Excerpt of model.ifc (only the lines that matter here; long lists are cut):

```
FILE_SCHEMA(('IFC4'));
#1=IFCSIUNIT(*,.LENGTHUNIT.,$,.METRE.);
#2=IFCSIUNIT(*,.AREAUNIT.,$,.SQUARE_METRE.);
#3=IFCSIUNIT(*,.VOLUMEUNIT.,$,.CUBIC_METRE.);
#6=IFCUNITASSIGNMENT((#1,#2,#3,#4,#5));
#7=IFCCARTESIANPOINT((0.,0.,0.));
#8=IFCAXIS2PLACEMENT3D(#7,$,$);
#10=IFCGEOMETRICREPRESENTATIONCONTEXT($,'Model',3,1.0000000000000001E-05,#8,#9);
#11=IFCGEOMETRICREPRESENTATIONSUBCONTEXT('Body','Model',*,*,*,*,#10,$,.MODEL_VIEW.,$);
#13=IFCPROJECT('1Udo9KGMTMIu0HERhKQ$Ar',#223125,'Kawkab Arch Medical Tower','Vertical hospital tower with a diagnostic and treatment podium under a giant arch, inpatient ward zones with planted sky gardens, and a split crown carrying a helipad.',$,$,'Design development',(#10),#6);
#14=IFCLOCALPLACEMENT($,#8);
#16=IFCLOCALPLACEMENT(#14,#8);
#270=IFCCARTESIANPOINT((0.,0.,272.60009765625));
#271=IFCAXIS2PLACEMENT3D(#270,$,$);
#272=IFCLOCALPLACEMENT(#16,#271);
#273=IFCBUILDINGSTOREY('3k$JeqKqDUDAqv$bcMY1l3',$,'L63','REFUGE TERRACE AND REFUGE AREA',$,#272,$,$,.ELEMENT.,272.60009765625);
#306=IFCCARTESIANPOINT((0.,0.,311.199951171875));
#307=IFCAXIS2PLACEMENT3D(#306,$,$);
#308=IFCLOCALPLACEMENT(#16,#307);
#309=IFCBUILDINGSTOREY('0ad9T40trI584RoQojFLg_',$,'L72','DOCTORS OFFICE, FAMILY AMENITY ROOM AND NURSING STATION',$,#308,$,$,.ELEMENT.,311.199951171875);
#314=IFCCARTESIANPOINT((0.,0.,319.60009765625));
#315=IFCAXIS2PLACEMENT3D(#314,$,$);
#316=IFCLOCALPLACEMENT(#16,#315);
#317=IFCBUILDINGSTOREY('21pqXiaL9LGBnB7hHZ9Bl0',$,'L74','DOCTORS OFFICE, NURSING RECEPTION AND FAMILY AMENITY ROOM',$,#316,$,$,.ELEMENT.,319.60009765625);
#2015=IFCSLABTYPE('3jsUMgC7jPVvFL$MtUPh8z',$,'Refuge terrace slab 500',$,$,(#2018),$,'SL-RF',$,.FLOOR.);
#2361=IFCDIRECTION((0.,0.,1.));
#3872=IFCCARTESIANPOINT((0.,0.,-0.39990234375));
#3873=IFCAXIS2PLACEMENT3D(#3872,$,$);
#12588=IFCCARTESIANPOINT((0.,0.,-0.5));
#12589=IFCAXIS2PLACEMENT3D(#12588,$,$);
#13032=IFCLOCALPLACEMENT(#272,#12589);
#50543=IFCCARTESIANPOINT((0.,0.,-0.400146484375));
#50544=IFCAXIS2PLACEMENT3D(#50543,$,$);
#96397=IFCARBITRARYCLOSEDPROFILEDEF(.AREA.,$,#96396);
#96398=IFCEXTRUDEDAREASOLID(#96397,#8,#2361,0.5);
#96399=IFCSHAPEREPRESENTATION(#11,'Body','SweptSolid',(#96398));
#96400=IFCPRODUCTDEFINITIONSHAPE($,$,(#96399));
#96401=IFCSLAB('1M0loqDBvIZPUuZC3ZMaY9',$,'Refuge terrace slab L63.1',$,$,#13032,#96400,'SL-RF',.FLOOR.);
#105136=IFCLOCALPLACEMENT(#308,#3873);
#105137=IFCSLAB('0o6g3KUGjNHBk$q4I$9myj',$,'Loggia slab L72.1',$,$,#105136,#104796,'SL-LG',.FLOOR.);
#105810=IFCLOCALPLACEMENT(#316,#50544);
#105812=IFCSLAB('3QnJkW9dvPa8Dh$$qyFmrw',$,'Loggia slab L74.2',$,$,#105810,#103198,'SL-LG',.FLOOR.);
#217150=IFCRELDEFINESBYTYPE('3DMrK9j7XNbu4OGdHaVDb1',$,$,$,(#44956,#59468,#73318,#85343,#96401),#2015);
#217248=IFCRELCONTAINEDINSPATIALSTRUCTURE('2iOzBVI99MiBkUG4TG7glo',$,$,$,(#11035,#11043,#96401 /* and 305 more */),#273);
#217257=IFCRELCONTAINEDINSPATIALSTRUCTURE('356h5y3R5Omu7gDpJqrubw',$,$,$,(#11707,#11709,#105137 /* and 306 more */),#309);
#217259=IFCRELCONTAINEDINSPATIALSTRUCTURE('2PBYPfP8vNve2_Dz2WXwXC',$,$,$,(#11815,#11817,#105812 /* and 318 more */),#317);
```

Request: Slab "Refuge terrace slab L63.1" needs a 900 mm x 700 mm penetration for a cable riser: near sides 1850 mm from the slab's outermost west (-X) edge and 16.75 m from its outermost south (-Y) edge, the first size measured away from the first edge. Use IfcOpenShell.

```python
import numpy as np
import ifcopenshell
import ifcopenshell.api.feature
import ifcopenshell.api.geometry
import ifcopenshell.api.root
import ifcopenshell.geom
import ifcopenshell.util.placement
import ifcopenshell.util.representation
import ifcopenshell.util.shape
import ifcopenshell.util.unit

model = ifcopenshell.open("model.ifc")
unit_scale = ifcopenshell.util.unit.calculate_unit_scale(model)
settings = ifcopenshell.geom.settings()


def volume(element):
    """Net volume in cubic metres, openings subtracted."""
    shape = ifcopenshell.geom.create_shape(settings, element)
    return ifcopenshell.util.shape.get_volume(shape.geometry)


slab = model.by_guid("1M0loqDBvIZPUuZC3ZMaY9")
before = volume(slab)

# Extent in the slab's own axes, in metres. The edges named are its -X and -Y sides.
slab_shape = ifcopenshell.geom.create_shape(settings, slab)
vertices = ifcopenshell.util.shape.get_vertices(slab_shape.geometry)
x_min, y_min, bottom = vertices.min(axis=0)
top = vertices[:, 2].max()

opening = ifcopenshell.api.root.create_entity(model, ifc_class="IfcOpeningElement", name="Cable riser opening", predefined_type="OPENING")
context = ifcopenshell.util.representation.get_context(model, "Model", "Body", "MODEL_VIEW")
width, depth = 0.9, 0.7
outline = [(0.0, 0.0), (width, 0.0), (width, depth), (0.0, depth), (0.0, 0.0)]
# Overshoot both faces by 50 mm so the cut is clean.
shape = ifcopenshell.api.geometry.add_slab_representation(
    model, context=context, depth=top - bottom + 0.1, polyline=outline
)
ifcopenshell.api.geometry.assign_representation(model, product=opening, representation=shape)

matrix = ifcopenshell.util.placement.get_local_placement(slab.ObjectPlacement)
matrix[:, 3] = matrix @ np.append(np.array([x_min + 1.85, y_min + 16.75, bottom - 0.05]) / unit_scale, 1.0)
ifcopenshell.api.geometry.edit_object_placement(model, product=opening, matrix=matrix, is_si=False)
ifcopenshell.api.feature.add_feature(model, feature=opening, element=slab)

after = volume(slab)

print(f"slab volume {before:.3f} -> {after:.3f} m3")

model.write("model_v2.ifc")
```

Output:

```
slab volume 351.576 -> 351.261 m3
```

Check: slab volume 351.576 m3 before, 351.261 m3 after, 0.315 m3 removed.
